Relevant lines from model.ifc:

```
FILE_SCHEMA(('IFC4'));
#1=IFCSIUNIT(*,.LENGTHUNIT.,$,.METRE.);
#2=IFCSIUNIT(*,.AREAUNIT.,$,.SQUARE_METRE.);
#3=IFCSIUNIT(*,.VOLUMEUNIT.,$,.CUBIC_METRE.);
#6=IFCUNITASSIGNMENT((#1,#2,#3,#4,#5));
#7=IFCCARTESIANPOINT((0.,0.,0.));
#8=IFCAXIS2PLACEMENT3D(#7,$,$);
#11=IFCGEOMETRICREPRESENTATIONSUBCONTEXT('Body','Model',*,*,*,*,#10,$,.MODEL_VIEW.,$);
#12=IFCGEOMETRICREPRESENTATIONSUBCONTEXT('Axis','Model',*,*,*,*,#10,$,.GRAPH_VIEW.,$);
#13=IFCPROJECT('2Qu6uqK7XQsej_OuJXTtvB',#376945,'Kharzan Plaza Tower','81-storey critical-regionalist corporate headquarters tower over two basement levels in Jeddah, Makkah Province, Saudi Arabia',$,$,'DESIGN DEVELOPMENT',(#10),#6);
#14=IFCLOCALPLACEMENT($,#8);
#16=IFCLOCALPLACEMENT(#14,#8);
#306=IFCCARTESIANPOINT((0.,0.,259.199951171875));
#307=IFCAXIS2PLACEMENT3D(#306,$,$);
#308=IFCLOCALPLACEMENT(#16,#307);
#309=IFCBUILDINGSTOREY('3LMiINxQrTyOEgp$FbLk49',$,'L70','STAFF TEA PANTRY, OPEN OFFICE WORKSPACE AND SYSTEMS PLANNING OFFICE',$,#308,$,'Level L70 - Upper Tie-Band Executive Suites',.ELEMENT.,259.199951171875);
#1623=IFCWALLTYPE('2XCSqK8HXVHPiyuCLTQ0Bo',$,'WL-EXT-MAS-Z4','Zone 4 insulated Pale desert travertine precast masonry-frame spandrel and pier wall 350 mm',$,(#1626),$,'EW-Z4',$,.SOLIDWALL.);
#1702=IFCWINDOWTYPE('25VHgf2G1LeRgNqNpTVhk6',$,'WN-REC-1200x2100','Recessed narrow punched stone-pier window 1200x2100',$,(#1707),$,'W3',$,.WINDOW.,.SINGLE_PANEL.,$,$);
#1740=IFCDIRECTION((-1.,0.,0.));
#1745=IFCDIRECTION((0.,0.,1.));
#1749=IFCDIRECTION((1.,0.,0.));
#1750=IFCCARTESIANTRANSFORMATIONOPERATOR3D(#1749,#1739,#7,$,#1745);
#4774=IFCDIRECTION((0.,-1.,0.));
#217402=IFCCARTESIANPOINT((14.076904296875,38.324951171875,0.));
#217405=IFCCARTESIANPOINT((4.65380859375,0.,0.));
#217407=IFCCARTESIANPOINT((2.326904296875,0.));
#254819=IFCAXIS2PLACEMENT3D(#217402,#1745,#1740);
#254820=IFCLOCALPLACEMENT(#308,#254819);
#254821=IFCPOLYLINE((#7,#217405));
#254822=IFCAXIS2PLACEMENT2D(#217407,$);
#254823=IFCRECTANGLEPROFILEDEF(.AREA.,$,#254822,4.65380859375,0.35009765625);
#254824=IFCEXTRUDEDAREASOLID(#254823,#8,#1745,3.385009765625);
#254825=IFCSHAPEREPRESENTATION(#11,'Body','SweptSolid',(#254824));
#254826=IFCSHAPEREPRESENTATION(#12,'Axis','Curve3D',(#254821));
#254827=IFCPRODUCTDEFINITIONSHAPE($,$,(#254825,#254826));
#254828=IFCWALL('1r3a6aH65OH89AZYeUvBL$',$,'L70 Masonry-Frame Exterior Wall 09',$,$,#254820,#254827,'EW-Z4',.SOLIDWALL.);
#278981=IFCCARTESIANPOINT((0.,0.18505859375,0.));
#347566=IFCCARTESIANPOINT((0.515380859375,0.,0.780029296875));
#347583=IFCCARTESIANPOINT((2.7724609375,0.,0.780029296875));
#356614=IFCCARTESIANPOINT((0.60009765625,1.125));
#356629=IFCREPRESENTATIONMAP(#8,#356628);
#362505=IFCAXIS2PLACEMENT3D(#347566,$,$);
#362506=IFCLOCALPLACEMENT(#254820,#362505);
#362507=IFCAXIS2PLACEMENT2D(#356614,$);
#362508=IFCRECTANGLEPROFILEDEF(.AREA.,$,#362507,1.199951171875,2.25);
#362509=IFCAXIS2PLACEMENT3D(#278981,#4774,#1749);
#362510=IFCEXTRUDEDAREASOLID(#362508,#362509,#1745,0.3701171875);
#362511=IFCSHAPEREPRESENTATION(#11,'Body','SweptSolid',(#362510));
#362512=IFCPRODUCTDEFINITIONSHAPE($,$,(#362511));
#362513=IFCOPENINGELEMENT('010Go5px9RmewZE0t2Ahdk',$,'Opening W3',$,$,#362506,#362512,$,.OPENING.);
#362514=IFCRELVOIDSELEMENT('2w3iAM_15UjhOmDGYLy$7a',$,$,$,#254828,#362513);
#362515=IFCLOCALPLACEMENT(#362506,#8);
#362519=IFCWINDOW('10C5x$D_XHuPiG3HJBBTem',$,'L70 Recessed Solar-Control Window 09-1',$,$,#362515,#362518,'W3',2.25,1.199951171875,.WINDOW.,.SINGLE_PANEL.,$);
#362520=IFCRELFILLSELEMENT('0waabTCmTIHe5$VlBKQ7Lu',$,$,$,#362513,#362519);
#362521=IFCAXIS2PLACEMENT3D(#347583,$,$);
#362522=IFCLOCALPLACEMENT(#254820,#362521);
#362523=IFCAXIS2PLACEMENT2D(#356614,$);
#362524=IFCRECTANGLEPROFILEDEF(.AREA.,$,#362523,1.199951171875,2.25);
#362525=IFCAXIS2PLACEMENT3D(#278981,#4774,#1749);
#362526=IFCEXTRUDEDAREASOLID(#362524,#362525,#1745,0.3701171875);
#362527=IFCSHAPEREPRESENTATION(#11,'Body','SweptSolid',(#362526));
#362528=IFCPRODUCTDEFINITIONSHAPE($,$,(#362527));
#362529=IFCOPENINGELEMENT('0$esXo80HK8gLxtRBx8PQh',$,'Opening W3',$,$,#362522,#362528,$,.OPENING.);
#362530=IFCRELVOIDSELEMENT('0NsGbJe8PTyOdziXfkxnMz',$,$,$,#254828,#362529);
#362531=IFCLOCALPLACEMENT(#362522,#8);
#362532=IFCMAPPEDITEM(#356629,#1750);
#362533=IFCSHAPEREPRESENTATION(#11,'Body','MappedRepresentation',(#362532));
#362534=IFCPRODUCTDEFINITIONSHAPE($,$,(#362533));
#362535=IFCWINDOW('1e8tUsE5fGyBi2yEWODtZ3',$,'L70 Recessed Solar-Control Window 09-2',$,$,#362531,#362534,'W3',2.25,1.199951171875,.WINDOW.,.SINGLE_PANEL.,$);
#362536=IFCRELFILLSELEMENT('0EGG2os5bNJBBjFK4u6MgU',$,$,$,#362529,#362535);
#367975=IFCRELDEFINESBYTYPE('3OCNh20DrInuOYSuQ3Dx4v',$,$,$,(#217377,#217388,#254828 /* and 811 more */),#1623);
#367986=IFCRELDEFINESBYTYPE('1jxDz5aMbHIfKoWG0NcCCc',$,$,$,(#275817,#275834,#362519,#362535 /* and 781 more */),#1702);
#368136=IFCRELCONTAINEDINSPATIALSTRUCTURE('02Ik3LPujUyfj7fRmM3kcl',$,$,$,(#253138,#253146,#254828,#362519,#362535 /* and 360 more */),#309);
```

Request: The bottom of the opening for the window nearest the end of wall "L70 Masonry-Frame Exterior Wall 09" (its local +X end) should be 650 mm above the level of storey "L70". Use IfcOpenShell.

```python
import numpy as np
import ifcopenshell
import ifcopenshell.api.geometry
import ifcopenshell.geom
import ifcopenshell.util.element
import ifcopenshell.util.placement
import ifcopenshell.util.shape
import ifcopenshell.util.unit

model = ifcopenshell.open("model.ifc")
unit_scale = ifcopenshell.util.unit.calculate_unit_scale(model)

window = model.by_guid("1e8tUsE5fGyBi2yEWODtZ3")
opening = window.FillsVoids[0].RelatingOpeningElement
storey = ifcopenshell.util.element.get_container(window, ifc_class="IfcBuildingStorey")
level = ifcopenshell.util.placement.get_local_placement(storey.ObjectPlacement)[2, 3]

# The opening's origin need not be at the sill, so measure its lowest point.
shape = ifcopenshell.geom.create_shape(ifcopenshell.geom.settings(), opening)
bottom = ifcopenshell.util.shape.get_shape_bottom_elevation(shape, shape.geometry) / unit_scale
dz = level + 0.65 - bottom

shift = np.array([0.0, 0.0, dz])
# The window is placed relative to its opening, so it follows when the opening moves.
matrix = ifcopenshell.util.placement.get_local_placement(opening.ObjectPlacement)
matrix[:3, 3] += shift
ifcopenshell.api.geometry.edit_object_placement(
    model, product=opening, matrix=matrix, is_si=False, should_transform_children=True
)

print(f"moved by {dz * unit_scale:+.3f} m")

model.write("model_rev.ifc")
```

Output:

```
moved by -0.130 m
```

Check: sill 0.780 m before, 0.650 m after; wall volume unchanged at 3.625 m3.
